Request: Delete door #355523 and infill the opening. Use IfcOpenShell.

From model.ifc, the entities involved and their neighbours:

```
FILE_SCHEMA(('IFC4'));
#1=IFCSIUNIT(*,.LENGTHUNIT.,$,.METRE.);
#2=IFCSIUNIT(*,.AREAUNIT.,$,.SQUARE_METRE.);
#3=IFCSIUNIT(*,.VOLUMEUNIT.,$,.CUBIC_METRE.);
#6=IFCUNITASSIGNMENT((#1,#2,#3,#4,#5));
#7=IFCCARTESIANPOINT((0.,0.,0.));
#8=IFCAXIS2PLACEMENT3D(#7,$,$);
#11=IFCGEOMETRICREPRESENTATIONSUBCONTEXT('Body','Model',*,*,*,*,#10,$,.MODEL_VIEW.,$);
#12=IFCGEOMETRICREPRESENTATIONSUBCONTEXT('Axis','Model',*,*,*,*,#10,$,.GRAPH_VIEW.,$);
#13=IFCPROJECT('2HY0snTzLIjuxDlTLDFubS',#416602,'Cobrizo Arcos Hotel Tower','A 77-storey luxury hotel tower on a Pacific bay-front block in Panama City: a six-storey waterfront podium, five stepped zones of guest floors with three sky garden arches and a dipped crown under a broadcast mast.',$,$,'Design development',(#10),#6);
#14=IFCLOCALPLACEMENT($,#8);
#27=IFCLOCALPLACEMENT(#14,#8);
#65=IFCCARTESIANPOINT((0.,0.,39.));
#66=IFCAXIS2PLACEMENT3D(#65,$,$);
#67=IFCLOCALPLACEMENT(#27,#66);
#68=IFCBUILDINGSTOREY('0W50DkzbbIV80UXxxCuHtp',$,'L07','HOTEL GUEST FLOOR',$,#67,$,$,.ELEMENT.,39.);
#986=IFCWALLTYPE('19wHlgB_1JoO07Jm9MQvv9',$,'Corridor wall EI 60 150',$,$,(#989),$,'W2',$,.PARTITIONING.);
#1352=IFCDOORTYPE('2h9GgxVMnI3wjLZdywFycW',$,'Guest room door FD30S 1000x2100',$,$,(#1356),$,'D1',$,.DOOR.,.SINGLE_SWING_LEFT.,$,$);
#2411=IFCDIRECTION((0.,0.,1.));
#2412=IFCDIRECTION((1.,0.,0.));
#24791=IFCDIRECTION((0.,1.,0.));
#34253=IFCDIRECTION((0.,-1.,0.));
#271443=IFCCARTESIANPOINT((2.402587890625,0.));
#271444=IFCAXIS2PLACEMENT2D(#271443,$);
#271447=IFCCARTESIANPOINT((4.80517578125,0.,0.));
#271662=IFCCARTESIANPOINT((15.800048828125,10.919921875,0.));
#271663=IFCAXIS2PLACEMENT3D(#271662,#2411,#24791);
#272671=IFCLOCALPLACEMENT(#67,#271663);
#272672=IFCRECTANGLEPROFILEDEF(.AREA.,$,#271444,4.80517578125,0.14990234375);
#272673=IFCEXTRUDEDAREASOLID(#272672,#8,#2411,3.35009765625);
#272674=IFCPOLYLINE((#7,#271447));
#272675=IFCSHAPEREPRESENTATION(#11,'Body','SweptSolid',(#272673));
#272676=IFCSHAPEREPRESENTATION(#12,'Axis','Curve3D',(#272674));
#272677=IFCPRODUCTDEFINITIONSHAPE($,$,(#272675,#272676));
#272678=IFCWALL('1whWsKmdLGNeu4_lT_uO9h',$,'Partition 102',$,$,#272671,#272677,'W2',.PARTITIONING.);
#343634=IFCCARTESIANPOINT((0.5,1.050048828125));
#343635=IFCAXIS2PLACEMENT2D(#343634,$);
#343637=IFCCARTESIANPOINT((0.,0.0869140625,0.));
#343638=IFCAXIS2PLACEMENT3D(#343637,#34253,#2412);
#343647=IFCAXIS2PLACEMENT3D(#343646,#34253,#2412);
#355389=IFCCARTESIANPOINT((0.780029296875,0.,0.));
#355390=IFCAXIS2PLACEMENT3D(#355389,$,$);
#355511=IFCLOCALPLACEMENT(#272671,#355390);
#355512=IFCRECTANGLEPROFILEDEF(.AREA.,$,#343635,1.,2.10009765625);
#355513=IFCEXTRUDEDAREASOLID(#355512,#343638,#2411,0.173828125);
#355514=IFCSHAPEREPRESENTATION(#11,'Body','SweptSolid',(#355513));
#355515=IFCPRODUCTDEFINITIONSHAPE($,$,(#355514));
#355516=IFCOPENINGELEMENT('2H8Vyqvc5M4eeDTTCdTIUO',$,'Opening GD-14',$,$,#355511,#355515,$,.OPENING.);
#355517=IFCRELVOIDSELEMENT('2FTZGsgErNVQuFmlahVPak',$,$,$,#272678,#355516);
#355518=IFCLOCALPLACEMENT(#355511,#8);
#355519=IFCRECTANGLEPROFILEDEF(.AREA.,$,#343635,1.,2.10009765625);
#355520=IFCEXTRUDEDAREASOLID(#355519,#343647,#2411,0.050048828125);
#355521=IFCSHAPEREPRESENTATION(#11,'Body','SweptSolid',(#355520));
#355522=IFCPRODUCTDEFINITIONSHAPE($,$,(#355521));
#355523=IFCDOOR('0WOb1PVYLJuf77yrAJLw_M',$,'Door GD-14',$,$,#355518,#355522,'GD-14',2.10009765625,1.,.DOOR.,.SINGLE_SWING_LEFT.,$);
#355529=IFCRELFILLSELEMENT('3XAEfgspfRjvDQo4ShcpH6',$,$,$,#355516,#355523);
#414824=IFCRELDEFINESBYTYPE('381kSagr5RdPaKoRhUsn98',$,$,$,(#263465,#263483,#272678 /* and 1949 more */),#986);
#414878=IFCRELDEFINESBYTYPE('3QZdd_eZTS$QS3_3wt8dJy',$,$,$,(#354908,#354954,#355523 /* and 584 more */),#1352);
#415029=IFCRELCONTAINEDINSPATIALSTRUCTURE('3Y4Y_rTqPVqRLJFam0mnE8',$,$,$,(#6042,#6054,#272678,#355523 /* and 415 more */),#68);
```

```python
import ifcopenshell
import ifcopenshell.api.feature
import ifcopenshell.api.root
import ifcopenshell.geom
import ifcopenshell.util.shape

model = ifcopenshell.open("model.ifc")
settings = ifcopenshell.geom.settings()


def volume(element):
    """Net volume in cubic metres, openings subtracted."""
    shape = ifcopenshell.geom.create_shape(settings, element)
    return ifcopenshell.util.shape.get_volume(shape.geometry)


door = model.by_guid("0WOb1PVYLJuf77yrAJLw_M")
opening = door.FillsVoids[0].RelatingOpeningElement
wall = opening.VoidsElements[0].RelatingBuildingElement
before = volume(wall)

ifcopenshell.api.root.remove_product(model, product=door)
ifcopenshell.api.feature.remove_feature(model, feature=opening)

after = volume(wall)

print(f"wall volume {before:.3f} -> {after:.3f} m3")

model.write("model_edited.ifc")
```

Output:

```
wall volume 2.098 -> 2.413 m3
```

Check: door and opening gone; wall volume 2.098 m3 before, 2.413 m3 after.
